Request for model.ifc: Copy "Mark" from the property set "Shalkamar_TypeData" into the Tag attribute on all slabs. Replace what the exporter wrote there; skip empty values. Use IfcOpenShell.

First a look at what the model holds.

```python
import ifcopenshell
import ifcopenshell.util.element

model = ifcopenshell.open("model.ifc")
print(model.schema)
slabs = model.by_type("IfcSlab")
print(len(slabs), "slabs")
for e in slabs[:8]:
    source = ifcopenshell.util.element.get_pset(e, "Shalkamar_TypeData", "Mark")
    target = e.Tag
    print(e.id(), repr(source), repr(target), sep=" | ")
```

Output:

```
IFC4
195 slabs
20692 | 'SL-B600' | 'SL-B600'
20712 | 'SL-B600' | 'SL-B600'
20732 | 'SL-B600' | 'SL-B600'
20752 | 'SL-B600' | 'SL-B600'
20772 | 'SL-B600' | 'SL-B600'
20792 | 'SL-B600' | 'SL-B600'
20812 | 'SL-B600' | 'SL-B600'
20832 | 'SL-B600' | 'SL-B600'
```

```python
import ifcopenshell
import ifcopenshell.util.element

model = ifcopenshell.open("model.ifc")

count = 0
for e in model.by_type("IfcSlab"):
    value = ifcopenshell.util.element.get_pset(e, "Shalkamar_TypeData", "Mark")
    current = e.Tag
    if not value or not value.strip() or current == value:
        continue
    e.Tag = value
    count += 1

print(count, "slabs updated")

model.write("model_updated.ifc")
```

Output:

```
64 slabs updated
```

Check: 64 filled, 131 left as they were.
